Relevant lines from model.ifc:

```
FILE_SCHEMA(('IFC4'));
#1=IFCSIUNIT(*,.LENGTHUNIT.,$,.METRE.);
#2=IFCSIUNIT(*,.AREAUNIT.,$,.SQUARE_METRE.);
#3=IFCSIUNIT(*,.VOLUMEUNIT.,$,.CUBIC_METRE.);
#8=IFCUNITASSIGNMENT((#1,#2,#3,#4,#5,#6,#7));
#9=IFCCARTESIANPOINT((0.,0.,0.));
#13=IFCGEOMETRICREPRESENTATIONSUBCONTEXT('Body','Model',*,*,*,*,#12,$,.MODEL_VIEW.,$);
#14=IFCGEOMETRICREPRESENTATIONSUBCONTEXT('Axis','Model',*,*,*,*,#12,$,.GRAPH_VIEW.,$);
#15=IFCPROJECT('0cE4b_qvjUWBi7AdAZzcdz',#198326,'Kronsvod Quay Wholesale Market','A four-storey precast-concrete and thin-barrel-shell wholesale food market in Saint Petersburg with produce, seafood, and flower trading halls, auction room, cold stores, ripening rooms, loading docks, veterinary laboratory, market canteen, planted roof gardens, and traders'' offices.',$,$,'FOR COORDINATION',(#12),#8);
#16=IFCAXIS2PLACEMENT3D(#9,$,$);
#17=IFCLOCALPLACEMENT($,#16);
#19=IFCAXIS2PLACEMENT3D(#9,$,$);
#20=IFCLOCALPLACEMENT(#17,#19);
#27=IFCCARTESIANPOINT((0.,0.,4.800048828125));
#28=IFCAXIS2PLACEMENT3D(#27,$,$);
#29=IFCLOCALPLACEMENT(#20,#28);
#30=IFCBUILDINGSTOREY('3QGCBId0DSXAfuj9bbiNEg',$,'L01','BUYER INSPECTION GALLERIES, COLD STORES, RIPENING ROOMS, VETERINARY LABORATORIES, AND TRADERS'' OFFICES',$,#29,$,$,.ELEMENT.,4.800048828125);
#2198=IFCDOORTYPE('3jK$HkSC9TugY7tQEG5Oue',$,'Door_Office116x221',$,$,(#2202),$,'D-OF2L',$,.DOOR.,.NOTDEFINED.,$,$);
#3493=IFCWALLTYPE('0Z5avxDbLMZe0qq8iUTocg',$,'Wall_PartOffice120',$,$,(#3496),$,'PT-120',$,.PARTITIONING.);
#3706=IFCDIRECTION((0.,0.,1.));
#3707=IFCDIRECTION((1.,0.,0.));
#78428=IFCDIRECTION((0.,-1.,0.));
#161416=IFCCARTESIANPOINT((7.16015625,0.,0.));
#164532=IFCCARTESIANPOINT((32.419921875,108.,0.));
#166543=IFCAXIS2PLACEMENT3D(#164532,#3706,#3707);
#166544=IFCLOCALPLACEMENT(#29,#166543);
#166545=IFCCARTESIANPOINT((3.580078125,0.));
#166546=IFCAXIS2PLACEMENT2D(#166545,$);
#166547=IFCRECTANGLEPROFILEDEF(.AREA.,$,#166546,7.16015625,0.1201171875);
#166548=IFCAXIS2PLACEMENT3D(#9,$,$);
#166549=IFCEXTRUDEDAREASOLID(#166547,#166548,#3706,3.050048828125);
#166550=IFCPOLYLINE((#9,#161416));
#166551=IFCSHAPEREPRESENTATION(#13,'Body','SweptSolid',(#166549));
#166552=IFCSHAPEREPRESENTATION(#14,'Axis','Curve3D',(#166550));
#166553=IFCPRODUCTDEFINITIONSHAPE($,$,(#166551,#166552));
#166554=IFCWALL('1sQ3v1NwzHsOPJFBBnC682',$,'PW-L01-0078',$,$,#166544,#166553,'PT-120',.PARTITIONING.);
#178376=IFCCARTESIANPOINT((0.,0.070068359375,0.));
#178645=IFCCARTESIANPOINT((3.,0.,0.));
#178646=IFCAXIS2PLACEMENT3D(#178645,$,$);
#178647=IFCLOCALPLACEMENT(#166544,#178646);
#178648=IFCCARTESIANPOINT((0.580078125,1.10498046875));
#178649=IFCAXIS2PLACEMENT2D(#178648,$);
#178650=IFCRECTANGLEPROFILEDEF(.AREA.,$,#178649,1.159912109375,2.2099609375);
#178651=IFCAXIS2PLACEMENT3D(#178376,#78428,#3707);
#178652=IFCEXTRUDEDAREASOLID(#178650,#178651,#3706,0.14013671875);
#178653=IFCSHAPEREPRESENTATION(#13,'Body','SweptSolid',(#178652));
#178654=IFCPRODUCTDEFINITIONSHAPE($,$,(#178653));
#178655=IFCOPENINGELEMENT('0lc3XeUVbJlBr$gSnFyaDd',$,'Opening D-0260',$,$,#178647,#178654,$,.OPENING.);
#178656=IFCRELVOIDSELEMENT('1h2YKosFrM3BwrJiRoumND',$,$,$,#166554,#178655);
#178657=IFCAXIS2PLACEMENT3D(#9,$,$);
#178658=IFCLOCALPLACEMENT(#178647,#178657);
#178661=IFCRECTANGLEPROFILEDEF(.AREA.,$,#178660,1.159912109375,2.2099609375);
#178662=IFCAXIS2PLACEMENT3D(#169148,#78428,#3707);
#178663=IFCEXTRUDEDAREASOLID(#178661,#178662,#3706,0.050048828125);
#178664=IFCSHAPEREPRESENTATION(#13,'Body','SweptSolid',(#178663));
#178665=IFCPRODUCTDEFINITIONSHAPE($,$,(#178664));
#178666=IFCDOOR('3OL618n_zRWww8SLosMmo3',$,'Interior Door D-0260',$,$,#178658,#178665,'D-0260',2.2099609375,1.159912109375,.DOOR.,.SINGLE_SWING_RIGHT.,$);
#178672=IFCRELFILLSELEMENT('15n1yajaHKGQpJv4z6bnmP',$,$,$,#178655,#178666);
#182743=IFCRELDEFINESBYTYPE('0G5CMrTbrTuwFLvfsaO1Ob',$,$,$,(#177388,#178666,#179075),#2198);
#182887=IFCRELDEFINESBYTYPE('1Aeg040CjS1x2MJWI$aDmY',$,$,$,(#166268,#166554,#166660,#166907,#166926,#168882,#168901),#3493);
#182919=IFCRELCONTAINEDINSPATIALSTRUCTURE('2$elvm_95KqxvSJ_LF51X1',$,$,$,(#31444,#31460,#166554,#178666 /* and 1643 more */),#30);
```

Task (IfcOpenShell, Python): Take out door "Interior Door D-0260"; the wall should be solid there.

```python
import ifcopenshell
import ifcopenshell.api.feature
import ifcopenshell.api.root
import ifcopenshell.geom
import ifcopenshell.util.shape

model = ifcopenshell.open("model.ifc")
settings = ifcopenshell.geom.settings()


def volume(element):
    """Net volume in cubic metres, openings subtracted."""
    shape = ifcopenshell.geom.create_shape(settings, element)
    return ifcopenshell.util.shape.get_volume(shape.geometry)


door = model.by_id(178666)
opening = door.FillsVoids[0].RelatingOpeningElement
wall = opening.VoidsElements[0].RelatingBuildingElement
before = volume(wall)

ifcopenshell.api.root.remove_product(model, product=door)
ifcopenshell.api.feature.remove_feature(model, feature=opening)

after = volume(wall)

print(f"wall volume {before:.3f} -> {after:.3f} m3")

model.write("model_updated.ifc")
```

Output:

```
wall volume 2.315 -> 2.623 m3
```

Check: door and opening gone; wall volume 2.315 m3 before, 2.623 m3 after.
